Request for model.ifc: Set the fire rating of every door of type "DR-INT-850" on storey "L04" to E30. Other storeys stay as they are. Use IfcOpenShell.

First a look at what the model holds.

```python
import ifcopenshell
import ifcopenshell.util.element

model = ifcopenshell.open("model.ifc")
print(model.schema)
storey = next(s for s in model.by_type("IfcBuildingStorey") if s.Name == "L04")
doors = [e for e in ifcopenshell.util.element.get_decomposition(storey) if e.is_a("IfcDoor")]
seen = {}
for e in doors:
    element_type = ifcopenshell.util.element.get_type(e)
    key = (element_type.Name if element_type != e and element_type else None, ifcopenshell.util.element.get_pset(e, "Pset_DoorCommon", "FireRating"))
    seen[key] = seen.get(key, 0) + 1
for (name, value), count in sorted(seen.items(), key=str):
    print(count, "x", name, "|", value)
```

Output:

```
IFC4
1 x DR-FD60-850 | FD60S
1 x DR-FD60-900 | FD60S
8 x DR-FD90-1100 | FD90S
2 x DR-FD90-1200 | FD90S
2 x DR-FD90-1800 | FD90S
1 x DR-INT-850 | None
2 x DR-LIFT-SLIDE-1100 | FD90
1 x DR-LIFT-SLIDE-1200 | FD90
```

```python
import ifcopenshell
import ifcopenshell.api.pset
import ifcopenshell.util.element

model = ifcopenshell.open("model.ifc")

storey = next(s for s in model.by_type("IfcBuildingStorey") if s.Name == "L04")
doors = [e for e in ifcopenshell.util.element.get_decomposition(storey) if e.is_a("IfcDoor")]

count = 0
for e in doors:
    element_type = ifcopenshell.util.element.get_type(e)
    if element_type in (None, e) or element_type.Name != "DR-INT-850":
        continue
    found = ifcopenshell.util.element.get_pset(e, "Pset_DoorCommon", should_inherit=False)
    if found:
        pset = model.by_id(found["id"])
        if len(ifcopenshell.util.element.get_elements_by_pset(pset)) > 1:
            pset = ifcopenshell.api.pset.unshare_pset(model, products=[e], pset=pset)[0]
    else:
        pset = ifcopenshell.api.pset.add_pset(model, product=e, name="Pset_DoorCommon")
    ifcopenshell.api.pset.edit_pset(model, pset=pset, properties={"FireRating": "E30"})
    count += 1

print(count, "doors updated")

model.write("model_v2.ifc")
```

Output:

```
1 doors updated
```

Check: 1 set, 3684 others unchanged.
